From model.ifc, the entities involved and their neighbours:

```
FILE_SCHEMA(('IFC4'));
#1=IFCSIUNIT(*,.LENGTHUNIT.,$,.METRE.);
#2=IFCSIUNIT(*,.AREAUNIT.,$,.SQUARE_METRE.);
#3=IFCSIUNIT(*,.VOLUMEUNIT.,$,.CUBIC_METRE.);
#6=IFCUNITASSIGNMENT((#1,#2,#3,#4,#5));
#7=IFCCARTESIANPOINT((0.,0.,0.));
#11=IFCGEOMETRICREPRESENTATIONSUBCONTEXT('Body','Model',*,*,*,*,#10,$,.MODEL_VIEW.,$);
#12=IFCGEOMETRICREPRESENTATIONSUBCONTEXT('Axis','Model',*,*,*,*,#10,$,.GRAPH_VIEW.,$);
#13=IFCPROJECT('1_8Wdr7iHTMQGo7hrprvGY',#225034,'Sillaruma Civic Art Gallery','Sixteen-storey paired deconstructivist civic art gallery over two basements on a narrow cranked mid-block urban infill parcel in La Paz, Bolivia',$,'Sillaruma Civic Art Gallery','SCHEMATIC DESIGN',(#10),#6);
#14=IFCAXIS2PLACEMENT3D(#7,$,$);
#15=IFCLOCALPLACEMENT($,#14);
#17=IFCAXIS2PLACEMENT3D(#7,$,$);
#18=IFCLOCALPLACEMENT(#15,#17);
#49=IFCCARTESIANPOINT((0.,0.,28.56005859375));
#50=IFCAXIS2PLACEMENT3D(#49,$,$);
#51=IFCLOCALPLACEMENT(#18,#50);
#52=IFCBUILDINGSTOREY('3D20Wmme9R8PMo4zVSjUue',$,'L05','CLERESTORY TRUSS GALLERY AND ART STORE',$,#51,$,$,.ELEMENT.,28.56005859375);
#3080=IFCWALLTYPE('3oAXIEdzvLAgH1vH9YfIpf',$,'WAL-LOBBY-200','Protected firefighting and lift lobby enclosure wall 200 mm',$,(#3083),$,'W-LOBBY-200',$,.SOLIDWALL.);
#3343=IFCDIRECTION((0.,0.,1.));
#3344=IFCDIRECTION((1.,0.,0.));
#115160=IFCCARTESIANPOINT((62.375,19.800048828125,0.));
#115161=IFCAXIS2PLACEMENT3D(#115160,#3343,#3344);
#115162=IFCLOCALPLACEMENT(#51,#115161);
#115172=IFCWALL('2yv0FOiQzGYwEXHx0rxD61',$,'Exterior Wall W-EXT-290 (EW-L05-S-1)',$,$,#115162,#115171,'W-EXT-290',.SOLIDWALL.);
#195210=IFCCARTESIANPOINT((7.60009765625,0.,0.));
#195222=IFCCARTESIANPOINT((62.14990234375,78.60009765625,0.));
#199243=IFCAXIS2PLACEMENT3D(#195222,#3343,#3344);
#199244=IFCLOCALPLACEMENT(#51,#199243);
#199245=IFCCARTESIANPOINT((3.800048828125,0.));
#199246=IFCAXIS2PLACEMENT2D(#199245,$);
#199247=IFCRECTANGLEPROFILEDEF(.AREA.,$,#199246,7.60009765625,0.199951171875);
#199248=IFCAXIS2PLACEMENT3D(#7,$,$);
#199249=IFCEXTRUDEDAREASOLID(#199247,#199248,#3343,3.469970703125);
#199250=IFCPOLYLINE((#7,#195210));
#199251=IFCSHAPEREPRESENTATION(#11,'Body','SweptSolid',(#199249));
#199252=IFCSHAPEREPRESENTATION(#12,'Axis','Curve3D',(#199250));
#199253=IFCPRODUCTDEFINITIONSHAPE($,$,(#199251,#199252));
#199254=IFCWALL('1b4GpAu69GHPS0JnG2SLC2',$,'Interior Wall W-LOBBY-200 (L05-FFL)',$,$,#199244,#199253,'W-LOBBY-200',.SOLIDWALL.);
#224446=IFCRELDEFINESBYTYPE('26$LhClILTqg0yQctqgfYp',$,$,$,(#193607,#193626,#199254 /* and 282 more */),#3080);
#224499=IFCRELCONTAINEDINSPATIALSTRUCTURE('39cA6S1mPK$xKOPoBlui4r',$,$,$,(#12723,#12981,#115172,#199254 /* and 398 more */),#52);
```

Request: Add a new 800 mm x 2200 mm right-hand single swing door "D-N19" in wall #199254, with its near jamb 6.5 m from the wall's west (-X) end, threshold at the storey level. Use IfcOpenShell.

```python
import numpy as np
import ifcopenshell
import ifcopenshell.api.feature
import ifcopenshell.api.geometry
import ifcopenshell.api.root
import ifcopenshell.api.spatial
import ifcopenshell.geom
import ifcopenshell.util.element
import ifcopenshell.util.placement
import ifcopenshell.util.representation
import ifcopenshell.util.shape
import ifcopenshell.util.unit

model = ifcopenshell.open("model.ifc")
unit_scale = ifcopenshell.util.unit.calculate_unit_scale(model)
settings = ifcopenshell.geom.settings()


def volume(element):
    """Net volume in cubic metres, openings subtracted."""
    shape = ifcopenshell.geom.create_shape(settings, element)
    return ifcopenshell.util.shape.get_volume(shape.geometry)


wall = model.by_guid("1b4GpAu69GHPS0JnG2SLC2")
storey = ifcopenshell.util.element.get_container(wall, ifc_class="IfcBuildingStorey")
context = ifcopenshell.util.representation.get_context(model, "Model", "Body", "MODEL_VIEW")
before = volume(wall)

width, height, from_end, sill = 0.8, 2.2, 6.5, 0.0  # metres

# The wall runs along its own X axis, and the end named is its -X end.
wall_shape = ifcopenshell.geom.create_shape(settings, wall)
x, y, z = ifcopenshell.util.shape.get_vertices(wall_shape.geometry).T
start = x.min() + from_end
face, thickness = float(y.min()), float(y.max() - y.min())
wall_matrix = ifcopenshell.util.placement.get_local_placement(wall.ObjectPlacement)
level = ifcopenshell.util.placement.get_local_placement(storey.ObjectPlacement)[2, 3]


def in_wall(x, y):
    """Placement at x, y metres in the wall's axes, at sill height."""
    matrix = wall_matrix.copy()
    matrix[:, 3] = wall_matrix @ np.array([x / unit_scale, y / unit_scale, 0.0, 1.0])
    matrix[2, 3] = level + sill / unit_scale
    return matrix


# Opening: a box that overshoots both wall faces by 50 mm.
opening = ifcopenshell.api.root.create_entity(model, ifc_class="IfcOpeningElement", predefined_type="OPENING")
box = ifcopenshell.api.geometry.add_wall_representation(
    model, context=context, length=width, height=height, thickness=thickness + 0.1
)
ifcopenshell.api.geometry.assign_representation(model, product=opening, representation=box)
ifcopenshell.api.geometry.edit_object_placement(model, product=opening, matrix=in_wall(start, face - 0.05), is_si=False)
ifcopenshell.api.feature.add_feature(model, feature=opening, element=wall)

door = ifcopenshell.api.root.create_entity(model, ifc_class="IfcDoor", name="D-N19", predefined_type="DOOR")
door.OverallWidth, door.OverallHeight = width / unit_scale, height / unit_scale
door.OperationType = "SINGLE_SWING_RIGHT"
body = ifcopenshell.api.geometry.add_door_representation(
    model,
    context=context,
    overall_width=door.OverallWidth,
    overall_height=door.OverallHeight,
    operation_type="SINGLE_SWING_RIGHT",
    lining_properties={"LiningDepth": thickness / unit_scale, "ThresholdDepth": thickness / unit_scale},
)
ifcopenshell.api.geometry.assign_representation(model, product=door, representation=body)
ifcopenshell.api.spatial.assign_container(model, products=[door], relating_structure=storey)
ifcopenshell.api.feature.add_filling(model, opening=opening, element=door)

# The lining spans the wall, so the door starts at the wall face.
ifcopenshell.api.geometry.edit_object_placement(model, product=door, matrix=in_wall(start, face), is_si=False)

after = volume(wall)

print(f"wall volume {before:.3f} -> {after:.3f} m3")

model.write("model_edited.ifc")
```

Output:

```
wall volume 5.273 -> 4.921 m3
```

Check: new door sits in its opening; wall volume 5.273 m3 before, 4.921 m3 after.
